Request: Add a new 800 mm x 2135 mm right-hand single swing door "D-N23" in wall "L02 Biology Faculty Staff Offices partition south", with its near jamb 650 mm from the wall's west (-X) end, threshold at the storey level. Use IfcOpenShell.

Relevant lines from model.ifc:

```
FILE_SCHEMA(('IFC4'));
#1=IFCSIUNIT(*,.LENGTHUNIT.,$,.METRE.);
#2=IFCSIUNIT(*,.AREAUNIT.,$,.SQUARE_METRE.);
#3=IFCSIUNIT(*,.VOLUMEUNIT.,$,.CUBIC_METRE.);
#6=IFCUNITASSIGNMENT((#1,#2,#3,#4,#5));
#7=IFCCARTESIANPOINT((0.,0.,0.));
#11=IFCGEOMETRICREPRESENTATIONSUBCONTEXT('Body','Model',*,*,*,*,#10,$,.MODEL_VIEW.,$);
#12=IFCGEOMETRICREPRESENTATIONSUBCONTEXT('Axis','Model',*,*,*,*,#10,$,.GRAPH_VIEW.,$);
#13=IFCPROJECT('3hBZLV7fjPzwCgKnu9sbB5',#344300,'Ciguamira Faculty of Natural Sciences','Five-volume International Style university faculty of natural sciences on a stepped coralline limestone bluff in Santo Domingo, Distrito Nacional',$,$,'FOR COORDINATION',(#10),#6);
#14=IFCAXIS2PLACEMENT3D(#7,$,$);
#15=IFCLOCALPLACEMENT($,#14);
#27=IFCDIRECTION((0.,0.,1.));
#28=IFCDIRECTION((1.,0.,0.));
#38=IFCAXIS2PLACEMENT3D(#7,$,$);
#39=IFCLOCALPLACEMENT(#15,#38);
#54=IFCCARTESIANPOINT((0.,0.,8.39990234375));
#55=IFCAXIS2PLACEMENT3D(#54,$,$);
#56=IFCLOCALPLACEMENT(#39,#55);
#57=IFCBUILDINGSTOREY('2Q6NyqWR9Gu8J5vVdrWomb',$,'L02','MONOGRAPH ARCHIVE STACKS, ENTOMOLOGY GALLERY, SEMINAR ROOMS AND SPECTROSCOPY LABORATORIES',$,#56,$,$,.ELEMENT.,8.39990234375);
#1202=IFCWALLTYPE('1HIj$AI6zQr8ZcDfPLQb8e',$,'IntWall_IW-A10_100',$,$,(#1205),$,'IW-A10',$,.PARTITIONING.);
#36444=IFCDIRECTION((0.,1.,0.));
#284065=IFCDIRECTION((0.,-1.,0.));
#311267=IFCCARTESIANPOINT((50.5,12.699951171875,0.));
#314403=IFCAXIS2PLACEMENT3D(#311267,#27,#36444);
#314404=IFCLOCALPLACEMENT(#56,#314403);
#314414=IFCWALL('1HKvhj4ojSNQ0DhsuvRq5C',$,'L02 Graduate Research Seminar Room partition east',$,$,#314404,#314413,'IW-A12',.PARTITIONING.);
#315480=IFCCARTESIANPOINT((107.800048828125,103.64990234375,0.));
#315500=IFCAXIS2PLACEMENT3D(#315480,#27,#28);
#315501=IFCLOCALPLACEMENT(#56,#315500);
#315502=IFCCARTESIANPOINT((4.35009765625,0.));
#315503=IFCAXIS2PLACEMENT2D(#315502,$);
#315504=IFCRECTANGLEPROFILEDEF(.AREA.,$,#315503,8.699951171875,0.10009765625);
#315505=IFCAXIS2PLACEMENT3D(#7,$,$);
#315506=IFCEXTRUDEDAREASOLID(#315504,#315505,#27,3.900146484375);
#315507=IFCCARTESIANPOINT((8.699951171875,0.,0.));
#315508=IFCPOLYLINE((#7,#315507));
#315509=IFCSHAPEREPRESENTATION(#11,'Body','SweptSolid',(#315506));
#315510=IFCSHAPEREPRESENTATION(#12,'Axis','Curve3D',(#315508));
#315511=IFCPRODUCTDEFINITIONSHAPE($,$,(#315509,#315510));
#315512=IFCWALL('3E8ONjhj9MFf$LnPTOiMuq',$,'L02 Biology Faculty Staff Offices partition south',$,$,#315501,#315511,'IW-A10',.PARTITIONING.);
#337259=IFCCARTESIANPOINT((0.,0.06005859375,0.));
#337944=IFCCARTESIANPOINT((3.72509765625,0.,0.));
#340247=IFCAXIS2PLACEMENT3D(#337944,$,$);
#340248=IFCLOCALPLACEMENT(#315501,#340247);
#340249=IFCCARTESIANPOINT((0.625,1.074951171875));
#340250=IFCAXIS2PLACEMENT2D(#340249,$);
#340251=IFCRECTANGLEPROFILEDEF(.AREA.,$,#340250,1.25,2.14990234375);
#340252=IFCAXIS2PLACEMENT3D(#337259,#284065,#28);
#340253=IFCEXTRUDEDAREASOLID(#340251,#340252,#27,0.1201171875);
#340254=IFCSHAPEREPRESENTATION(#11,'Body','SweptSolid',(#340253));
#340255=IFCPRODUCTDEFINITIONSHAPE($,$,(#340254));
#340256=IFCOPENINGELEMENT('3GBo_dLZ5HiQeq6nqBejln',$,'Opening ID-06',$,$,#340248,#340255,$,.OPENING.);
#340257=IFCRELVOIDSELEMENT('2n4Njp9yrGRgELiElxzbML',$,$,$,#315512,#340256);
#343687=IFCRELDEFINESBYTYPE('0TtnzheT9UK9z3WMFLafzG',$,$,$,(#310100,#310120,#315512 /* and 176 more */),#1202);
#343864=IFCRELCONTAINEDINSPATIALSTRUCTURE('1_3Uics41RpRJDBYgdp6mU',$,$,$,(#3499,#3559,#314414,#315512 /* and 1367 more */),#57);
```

```python
import numpy as np
import ifcopenshell
import ifcopenshell.api.feature
import ifcopenshell.api.geometry
import ifcopenshell.api.root
import ifcopenshell.api.spatial
import ifcopenshell.geom
import ifcopenshell.util.element
import ifcopenshell.util.placement
import ifcopenshell.util.representation
import ifcopenshell.util.shape
import ifcopenshell.util.unit

model = ifcopenshell.open("model.ifc")
unit_scale = ifcopenshell.util.unit.calculate_unit_scale(model)
settings = ifcopenshell.geom.settings()


def volume(element):
    """Net volume in cubic metres, openings subtracted."""
    shape = ifcopenshell.geom.create_shape(settings, element)
    return ifcopenshell.util.shape.get_volume(shape.geometry)


wall = model.by_id(315512)
storey = ifcopenshell.util.element.get_container(wall, ifc_class="IfcBuildingStorey")
context = ifcopenshell.util.representation.get_context(model, "Model", "Body", "MODEL_VIEW")
before = volume(wall)

width, height, from_end, sill = 0.8, 2.135, 0.65, 0.0  # metres

# The wall runs along its own X axis, and the end named is its -X end.
wall_shape = ifcopenshell.geom.create_shape(settings, wall)
x, y, z = ifcopenshell.util.shape.get_vertices(wall_shape.geometry).T
start = x.min() + from_end
face, thickness = float(y.min()), float(y.max() - y.min())
wall_matrix = ifcopenshell.util.placement.get_local_placement(wall.ObjectPlacement)
level = ifcopenshell.util.placement.get_local_placement(storey.ObjectPlacement)[2, 3]


def in_wall(x, y):
    """Placement at x, y metres in the wall's axes, at sill height."""
    matrix = wall_matrix.copy()
    matrix[:, 3] = wall_matrix @ np.array([x / unit_scale, y / unit_scale, 0.0, 1.0])
    matrix[2, 3] = level + sill / unit_scale
    return matrix


# Opening: a box that overshoots both wall faces by 50 mm.
opening = ifcopenshell.api.root.create_entity(model, ifc_class="IfcOpeningElement", predefined_type="OPENING")
box = ifcopenshell.api.geometry.add_wall_representation(
    model, context=context, length=width, height=height, thickness=thickness + 0.1
)
ifcopenshell.api.geometry.assign_representation(model, product=opening, representation=box)
ifcopenshell.api.geometry.edit_object_placement(model, product=opening, matrix=in_wall(start, face - 0.05), is_si=False)
ifcopenshell.api.feature.add_feature(model, feature=opening, element=wall)

door = ifcopenshell.api.root.create_entity(model, ifc_class="IfcDoor", name="D-N23", predefined_type="DOOR")
door.OverallWidth, door.OverallHeight = width / unit_scale, height / unit_scale
door.OperationType = "SINGLE_SWING_RIGHT"
body = ifcopenshell.api.geometry.add_door_representation(
    model,
    context=context,
    overall_width=door.OverallWidth,
    overall_height=door.OverallHeight,
    operation_type="SINGLE_SWING_RIGHT",
    lining_properties={"LiningDepth": thickness / unit_scale, "ThresholdDepth": thickness / unit_scale},
)
ifcopenshell.api.geometry.assign_representation(model, product=door, representation=body)
ifcopenshell.api.spatial.assign_container(model, products=[door], relating_structure=storey)
ifcopenshell.api.feature.add_filling(model, opening=opening, element=door)

# The lining spans the wall, so the door starts at the wall face.
ifcopenshell.api.geometry.edit_object_placement(model, product=door, matrix=in_wall(start, face), is_si=False)

after = volume(wall)

print(f"wall volume {before:.3f} -> {after:.3f} m3")

model.write("model-out.ifc")
```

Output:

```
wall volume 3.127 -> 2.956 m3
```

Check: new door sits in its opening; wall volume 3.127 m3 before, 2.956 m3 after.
